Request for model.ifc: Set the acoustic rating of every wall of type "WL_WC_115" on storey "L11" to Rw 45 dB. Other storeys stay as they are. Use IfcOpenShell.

First a look at what the model holds.

```python
import ifcopenshell
import ifcopenshell.util.element

model = ifcopenshell.open("model.ifc")
print(model.schema)
storey = next(s for s in model.by_type("IfcBuildingStorey") if s.Name == "L11")
walls = [e for e in ifcopenshell.util.element.get_decomposition(storey) if e.is_a("IfcWall")]
seen = {}
for e in walls:
    element_type = ifcopenshell.util.element.get_type(e)
    key = (element_type.Name if element_type != e and element_type else None, ifcopenshell.util.element.get_pset(e, "Pset_WallCommon", "AcousticRating"))
    seen[key] = seen.get(key, 0) + 1
for (name, value), count in sorted(seen.items(), key=str):
    print(count, "x", name, "|", value)
```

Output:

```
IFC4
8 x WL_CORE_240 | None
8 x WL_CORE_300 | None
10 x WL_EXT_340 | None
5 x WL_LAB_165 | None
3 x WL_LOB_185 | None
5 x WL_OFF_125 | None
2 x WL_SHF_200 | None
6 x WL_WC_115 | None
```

```python
import ifcopenshell
import ifcopenshell.api.pset
import ifcopenshell.util.element

model = ifcopenshell.open("model.ifc")

storey = next(s for s in model.by_type("IfcBuildingStorey") if s.Name == "L11")
walls = [e for e in ifcopenshell.util.element.get_decomposition(storey) if e.is_a("IfcWall")]

count = 0
for e in walls:
    element_type = ifcopenshell.util.element.get_type(e)
    if element_type in (None, e) or element_type.Name != "WL_WC_115":
        continue
    # add_pset returns the element's existing set when there is one.
    pset = ifcopenshell.api.pset.add_pset(model, product=e, name="Pset_WallCommon")
    ifcopenshell.api.pset.edit_pset(model, pset=pset, properties={"AcousticRating": "Rw 45 dB"})
    count += 1

print(count, "walls updated")

model.write("model-out.ifc")
```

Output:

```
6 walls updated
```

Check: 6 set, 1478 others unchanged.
